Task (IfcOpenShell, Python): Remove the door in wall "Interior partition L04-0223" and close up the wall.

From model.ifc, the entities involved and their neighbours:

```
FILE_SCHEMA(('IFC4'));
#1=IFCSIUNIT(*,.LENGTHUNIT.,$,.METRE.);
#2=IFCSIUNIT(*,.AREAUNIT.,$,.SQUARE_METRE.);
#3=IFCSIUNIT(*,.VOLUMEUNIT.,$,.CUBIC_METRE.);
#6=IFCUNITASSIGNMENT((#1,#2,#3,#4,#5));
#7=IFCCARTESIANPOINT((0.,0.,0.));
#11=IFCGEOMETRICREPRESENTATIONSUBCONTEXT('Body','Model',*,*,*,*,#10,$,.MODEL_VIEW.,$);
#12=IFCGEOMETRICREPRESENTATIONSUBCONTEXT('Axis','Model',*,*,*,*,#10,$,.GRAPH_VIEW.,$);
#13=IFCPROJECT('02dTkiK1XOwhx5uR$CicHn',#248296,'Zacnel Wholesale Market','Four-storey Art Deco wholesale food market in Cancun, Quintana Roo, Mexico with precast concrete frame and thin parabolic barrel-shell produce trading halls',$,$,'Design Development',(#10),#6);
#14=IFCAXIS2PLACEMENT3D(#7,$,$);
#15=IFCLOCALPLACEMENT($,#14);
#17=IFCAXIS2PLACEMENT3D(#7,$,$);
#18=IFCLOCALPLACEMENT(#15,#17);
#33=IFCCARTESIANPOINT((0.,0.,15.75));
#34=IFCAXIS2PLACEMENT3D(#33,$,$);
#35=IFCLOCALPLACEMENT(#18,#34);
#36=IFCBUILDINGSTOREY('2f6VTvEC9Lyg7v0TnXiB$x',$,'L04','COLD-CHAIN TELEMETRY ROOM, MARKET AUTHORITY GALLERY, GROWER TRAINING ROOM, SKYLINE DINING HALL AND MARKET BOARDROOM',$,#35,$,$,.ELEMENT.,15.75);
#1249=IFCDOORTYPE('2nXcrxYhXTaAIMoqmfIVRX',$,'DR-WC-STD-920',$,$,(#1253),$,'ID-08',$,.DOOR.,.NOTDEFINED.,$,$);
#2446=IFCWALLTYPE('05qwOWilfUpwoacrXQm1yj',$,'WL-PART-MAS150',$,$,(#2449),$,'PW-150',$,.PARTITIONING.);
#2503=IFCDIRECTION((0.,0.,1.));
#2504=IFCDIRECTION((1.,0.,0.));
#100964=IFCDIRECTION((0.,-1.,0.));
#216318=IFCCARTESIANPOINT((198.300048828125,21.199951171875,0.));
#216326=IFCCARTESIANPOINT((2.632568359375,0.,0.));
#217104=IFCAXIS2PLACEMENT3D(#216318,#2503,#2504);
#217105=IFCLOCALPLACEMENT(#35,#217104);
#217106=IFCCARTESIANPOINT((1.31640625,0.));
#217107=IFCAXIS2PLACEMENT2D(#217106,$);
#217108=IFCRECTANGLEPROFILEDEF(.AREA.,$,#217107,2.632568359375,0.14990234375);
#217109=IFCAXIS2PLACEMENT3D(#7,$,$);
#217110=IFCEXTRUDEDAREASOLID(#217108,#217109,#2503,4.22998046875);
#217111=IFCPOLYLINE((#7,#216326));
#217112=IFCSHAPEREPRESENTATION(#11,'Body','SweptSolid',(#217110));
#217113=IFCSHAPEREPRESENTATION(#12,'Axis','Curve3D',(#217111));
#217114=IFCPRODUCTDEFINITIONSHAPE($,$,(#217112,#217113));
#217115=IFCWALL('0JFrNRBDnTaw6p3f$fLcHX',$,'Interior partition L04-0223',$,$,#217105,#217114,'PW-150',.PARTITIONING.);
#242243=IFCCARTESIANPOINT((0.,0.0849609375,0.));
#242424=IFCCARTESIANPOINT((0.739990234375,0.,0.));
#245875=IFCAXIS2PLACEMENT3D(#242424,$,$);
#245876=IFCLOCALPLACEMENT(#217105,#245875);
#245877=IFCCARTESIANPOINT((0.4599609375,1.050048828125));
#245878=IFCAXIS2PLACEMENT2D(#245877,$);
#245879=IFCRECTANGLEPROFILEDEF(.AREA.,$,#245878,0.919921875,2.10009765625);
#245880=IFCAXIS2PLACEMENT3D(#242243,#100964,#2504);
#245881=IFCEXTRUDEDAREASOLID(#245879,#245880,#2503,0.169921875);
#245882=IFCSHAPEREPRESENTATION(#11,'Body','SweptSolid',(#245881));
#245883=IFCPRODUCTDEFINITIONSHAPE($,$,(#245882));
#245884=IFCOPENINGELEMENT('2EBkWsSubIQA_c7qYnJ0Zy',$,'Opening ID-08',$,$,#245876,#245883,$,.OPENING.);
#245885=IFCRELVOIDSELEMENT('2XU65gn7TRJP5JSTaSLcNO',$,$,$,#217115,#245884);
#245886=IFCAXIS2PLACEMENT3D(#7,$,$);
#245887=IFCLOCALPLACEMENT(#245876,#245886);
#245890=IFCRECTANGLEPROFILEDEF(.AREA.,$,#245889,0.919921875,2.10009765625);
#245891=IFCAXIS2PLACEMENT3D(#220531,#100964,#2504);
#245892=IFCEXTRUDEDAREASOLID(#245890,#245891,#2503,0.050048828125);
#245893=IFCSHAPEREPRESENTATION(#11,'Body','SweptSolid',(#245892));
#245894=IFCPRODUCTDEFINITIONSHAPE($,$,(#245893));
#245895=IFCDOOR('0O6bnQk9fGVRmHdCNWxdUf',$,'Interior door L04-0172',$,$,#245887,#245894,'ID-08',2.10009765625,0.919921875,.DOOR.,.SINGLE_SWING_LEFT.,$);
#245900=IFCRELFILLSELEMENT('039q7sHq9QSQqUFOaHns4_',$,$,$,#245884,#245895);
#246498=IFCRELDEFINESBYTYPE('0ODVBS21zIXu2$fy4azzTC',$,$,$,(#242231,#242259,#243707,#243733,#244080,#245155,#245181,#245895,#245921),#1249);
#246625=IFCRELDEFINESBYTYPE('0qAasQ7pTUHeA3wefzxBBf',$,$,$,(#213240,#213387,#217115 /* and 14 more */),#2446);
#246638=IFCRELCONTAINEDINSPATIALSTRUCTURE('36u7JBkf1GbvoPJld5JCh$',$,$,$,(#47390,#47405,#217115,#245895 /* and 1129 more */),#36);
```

```python
import ifcopenshell
import ifcopenshell.api.feature
import ifcopenshell.api.root
import ifcopenshell.geom
import ifcopenshell.util.shape

model = ifcopenshell.open("model.ifc")
settings = ifcopenshell.geom.settings()


def volume(element):
    """Net volume in cubic metres, openings subtracted."""
    shape = ifcopenshell.geom.create_shape(settings, element)
    return ifcopenshell.util.shape.get_volume(shape.geometry)


door = model.by_guid("0O6bnQk9fGVRmHdCNWxdUf")
opening = door.FillsVoids[0].RelatingOpeningElement
wall = opening.VoidsElements[0].RelatingBuildingElement
before = volume(wall)

ifcopenshell.api.root.remove_product(model, product=door)
ifcopenshell.api.feature.remove_feature(model, feature=opening)

after = volume(wall)

print(f"wall volume {before:.3f} -> {after:.3f} m3")

model.write("model_edited.ifc")
```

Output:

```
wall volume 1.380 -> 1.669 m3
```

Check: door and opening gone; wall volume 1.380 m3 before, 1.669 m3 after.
